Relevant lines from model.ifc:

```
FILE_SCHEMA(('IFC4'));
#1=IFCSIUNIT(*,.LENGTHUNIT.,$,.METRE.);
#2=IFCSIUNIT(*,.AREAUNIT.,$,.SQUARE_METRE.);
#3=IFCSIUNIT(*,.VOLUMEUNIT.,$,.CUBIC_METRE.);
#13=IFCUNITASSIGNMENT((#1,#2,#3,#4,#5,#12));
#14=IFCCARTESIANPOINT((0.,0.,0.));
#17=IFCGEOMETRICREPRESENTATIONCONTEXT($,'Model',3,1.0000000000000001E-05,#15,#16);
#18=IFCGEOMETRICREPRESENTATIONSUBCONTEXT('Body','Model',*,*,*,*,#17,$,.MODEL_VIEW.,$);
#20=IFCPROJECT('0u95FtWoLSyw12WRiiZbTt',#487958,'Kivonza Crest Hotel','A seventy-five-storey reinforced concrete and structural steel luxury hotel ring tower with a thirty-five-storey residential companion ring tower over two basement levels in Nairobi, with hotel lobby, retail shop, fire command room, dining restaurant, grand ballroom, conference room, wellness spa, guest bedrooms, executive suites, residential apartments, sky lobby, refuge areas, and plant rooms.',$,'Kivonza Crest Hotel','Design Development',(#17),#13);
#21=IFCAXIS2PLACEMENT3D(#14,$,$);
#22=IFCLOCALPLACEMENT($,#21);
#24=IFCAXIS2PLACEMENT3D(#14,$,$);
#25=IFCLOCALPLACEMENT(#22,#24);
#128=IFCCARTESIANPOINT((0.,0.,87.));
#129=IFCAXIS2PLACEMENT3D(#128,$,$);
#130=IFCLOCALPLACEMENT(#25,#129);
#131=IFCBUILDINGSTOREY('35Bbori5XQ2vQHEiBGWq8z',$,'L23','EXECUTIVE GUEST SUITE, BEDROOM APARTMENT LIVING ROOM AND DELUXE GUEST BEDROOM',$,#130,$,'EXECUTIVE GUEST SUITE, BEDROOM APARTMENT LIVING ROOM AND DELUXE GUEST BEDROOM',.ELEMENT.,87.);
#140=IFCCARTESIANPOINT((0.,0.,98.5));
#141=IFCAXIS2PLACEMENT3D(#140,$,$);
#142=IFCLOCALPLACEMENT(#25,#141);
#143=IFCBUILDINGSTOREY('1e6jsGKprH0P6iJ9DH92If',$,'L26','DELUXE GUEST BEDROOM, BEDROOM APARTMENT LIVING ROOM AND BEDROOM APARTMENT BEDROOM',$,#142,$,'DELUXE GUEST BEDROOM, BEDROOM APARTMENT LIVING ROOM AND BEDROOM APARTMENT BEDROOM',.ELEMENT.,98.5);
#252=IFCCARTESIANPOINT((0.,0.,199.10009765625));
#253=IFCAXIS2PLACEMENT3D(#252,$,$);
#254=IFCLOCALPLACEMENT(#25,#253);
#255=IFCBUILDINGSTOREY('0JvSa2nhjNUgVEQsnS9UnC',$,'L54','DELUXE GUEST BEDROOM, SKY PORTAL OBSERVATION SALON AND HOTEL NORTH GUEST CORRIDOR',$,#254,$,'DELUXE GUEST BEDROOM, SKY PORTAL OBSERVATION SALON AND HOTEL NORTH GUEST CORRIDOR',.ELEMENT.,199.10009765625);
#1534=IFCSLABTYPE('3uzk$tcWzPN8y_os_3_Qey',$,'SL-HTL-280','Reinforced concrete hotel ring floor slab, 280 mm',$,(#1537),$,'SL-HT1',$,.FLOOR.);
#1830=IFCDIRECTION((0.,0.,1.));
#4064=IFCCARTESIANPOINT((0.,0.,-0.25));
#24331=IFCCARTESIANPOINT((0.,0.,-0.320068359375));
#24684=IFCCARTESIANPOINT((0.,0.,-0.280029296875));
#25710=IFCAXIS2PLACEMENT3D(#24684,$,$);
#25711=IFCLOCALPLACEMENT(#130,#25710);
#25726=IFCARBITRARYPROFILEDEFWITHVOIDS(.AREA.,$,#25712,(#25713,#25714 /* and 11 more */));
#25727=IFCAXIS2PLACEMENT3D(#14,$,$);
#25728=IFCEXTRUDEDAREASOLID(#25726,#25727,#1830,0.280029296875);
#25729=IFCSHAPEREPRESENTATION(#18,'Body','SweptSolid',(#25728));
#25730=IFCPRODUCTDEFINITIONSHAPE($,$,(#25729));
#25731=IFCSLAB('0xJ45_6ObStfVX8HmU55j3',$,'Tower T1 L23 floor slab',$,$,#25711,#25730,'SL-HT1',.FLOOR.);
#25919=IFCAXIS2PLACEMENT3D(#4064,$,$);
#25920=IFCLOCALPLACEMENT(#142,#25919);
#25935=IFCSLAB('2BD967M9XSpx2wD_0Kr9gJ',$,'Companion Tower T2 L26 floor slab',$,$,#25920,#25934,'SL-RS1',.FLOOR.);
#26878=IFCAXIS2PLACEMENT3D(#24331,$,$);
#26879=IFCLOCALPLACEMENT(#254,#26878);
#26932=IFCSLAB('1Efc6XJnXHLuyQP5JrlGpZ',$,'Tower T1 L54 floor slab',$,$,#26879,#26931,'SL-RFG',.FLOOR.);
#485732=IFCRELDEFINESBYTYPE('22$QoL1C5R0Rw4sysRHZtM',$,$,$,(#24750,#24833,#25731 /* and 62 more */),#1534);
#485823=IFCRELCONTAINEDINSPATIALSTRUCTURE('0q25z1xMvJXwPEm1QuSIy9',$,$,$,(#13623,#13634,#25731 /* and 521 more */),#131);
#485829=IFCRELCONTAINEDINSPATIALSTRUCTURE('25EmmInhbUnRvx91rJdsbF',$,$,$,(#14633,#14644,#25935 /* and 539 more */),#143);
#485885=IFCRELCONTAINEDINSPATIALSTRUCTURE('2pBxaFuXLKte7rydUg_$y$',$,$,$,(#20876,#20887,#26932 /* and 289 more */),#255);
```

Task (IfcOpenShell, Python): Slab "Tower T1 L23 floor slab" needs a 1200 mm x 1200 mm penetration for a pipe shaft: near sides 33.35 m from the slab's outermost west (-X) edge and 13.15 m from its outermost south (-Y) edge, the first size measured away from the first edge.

```python
import numpy as np
import ifcopenshell
import ifcopenshell.api.feature
import ifcopenshell.api.geometry
import ifcopenshell.api.root
import ifcopenshell.geom
import ifcopenshell.util.placement
import ifcopenshell.util.representation
import ifcopenshell.util.shape
import ifcopenshell.util.unit

model = ifcopenshell.open("model.ifc")
unit_scale = ifcopenshell.util.unit.calculate_unit_scale(model)
settings = ifcopenshell.geom.settings()


def volume(element):
    """Net volume in cubic metres, openings subtracted."""
    shape = ifcopenshell.geom.create_shape(settings, element)
    return ifcopenshell.util.shape.get_volume(shape.geometry)


slab = model.by_guid("0xJ45_6ObStfVX8HmU55j3")
before = volume(slab)

# Extent in the slab's own axes, in metres. The edges named are its -X and -Y sides.
slab_shape = ifcopenshell.geom.create_shape(settings, slab)
vertices = ifcopenshell.util.shape.get_vertices(slab_shape.geometry)
x_min, y_min, bottom = vertices.min(axis=0)
top = vertices[:, 2].max()

opening = ifcopenshell.api.root.create_entity(model, ifc_class="IfcOpeningElement", name="Pipe shaft opening", predefined_type="OPENING")
context = ifcopenshell.util.representation.get_context(model, "Model", "Body", "MODEL_VIEW")
width, depth = 1.2, 1.2
outline = [(0.0, 0.0), (width, 0.0), (width, depth), (0.0, depth), (0.0, 0.0)]
# Overshoot both faces by 50 mm so the cut is clean.
shape = ifcopenshell.api.geometry.add_slab_representation(
    model, context=context, depth=top - bottom + 0.1, polyline=outline
)
ifcopenshell.api.geometry.assign_representation(model, product=opening, representation=shape)

matrix = ifcopenshell.util.placement.get_local_placement(slab.ObjectPlacement)
matrix[:, 3] = matrix @ np.append(np.array([x_min + 33.35, y_min + 13.15, bottom - 0.05]) / unit_scale, 1.0)
ifcopenshell.api.geometry.edit_object_placement(model, product=opening, matrix=matrix, is_si=False)
ifcopenshell.api.feature.add_feature(model, feature=opening, element=slab)

after = volume(slab)

print(f"slab volume {before:.3f} -> {after:.3f} m3")

model.write("model-out.ifc")
```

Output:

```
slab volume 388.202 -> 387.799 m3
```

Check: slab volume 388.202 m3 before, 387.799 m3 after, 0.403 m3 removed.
